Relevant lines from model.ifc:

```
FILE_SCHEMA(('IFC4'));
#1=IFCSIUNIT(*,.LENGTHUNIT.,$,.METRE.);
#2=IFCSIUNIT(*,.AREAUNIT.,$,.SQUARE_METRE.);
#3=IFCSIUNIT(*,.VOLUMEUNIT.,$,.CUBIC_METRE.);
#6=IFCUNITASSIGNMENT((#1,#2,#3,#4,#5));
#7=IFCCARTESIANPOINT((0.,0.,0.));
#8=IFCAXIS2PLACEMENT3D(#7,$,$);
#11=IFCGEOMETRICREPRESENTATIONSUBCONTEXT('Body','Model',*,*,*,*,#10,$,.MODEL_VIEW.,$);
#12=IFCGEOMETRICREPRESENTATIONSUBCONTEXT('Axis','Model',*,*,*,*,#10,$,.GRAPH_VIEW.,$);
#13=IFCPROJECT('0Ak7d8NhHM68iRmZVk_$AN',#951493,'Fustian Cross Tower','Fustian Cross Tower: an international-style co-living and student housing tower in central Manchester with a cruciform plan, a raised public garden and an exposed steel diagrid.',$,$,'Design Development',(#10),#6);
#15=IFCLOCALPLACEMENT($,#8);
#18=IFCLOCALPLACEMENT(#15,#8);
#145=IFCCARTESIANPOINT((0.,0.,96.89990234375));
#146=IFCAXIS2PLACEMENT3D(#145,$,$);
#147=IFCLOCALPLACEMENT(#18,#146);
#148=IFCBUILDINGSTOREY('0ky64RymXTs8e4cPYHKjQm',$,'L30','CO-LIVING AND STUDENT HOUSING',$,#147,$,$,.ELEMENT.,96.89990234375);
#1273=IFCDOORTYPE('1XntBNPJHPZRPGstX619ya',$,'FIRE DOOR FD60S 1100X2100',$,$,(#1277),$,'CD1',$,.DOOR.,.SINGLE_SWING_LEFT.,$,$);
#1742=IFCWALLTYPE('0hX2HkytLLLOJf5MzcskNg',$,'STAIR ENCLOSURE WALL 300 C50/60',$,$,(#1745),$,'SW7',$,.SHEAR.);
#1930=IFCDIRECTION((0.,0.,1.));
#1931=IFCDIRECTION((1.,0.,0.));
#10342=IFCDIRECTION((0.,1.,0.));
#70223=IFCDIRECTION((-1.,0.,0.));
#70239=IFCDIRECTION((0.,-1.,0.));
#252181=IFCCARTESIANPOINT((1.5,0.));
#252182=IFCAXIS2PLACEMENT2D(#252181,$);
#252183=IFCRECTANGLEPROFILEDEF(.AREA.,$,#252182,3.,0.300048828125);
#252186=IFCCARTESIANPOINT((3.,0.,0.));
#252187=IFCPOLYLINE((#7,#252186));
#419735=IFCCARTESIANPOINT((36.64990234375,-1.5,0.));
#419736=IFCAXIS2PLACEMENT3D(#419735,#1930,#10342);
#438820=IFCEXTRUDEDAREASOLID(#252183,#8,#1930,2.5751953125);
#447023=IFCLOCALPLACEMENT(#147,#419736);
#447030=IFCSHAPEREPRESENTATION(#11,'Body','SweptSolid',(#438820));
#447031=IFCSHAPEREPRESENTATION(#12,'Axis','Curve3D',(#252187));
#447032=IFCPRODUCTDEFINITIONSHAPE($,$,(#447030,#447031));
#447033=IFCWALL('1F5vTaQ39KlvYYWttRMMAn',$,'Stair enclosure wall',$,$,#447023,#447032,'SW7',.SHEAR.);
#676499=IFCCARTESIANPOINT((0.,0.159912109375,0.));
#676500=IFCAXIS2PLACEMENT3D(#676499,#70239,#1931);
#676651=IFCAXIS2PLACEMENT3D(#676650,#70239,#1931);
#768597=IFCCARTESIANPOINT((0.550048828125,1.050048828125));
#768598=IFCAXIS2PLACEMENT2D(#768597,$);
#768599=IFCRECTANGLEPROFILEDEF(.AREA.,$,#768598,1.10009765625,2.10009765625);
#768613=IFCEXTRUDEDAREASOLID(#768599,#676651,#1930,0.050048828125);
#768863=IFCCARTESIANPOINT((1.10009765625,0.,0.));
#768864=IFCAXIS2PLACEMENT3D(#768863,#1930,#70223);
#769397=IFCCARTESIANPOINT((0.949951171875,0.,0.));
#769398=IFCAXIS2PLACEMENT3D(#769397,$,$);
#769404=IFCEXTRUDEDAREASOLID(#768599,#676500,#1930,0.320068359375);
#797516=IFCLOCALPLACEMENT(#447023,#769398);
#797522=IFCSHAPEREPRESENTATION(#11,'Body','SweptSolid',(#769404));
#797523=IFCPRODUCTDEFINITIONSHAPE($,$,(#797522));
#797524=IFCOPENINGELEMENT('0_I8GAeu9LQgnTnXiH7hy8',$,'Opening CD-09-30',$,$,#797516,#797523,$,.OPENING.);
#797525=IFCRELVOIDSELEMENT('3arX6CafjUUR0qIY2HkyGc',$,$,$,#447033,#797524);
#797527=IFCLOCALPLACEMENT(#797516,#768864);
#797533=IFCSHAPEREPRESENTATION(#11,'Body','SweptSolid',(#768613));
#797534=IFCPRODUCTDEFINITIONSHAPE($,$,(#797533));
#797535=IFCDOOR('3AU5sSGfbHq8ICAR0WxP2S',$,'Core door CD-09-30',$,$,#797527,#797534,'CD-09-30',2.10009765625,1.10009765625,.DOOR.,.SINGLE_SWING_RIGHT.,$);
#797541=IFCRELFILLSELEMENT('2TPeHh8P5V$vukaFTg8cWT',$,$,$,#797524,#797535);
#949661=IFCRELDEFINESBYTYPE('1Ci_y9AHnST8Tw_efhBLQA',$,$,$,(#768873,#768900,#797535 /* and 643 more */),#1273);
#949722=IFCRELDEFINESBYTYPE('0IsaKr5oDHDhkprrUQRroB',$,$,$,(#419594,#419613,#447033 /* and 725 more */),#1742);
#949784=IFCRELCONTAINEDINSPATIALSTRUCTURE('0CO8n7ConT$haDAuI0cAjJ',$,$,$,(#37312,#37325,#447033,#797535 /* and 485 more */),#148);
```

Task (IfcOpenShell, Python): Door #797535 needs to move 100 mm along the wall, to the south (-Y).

```python
import ifcopenshell
import ifcopenshell.api.geometry
import ifcopenshell.util.placement
import ifcopenshell.util.unit

model = ifcopenshell.open("model.ifc")
unit_scale = ifcopenshell.util.unit.calculate_unit_scale(model)

door = model.by_guid("3AU5sSGfbHq8ICAR0WxP2S")
opening = door.FillsVoids[0].RelatingOpeningElement
wall = opening.VoidsElements[0].RelatingBuildingElement

wall_matrix = ifcopenshell.util.placement.get_local_placement(wall.ObjectPlacement)
shift = wall_matrix[:3, 0] * -0.1 / unit_scale
before = ifcopenshell.util.placement.get_local_placement(door.ObjectPlacement)[:3, 3].copy()

# The door is placed relative to its opening, so it follows when the opening moves.
matrix = ifcopenshell.util.placement.get_local_placement(opening.ObjectPlacement)
matrix[:3, 3] += shift
ifcopenshell.api.geometry.edit_object_placement(
    model, product=opening, matrix=matrix, is_si=False, should_transform_children=True
)

after = ifcopenshell.util.placement.get_local_placement(door.ObjectPlacement)[:3, 3]
print("door moved by", (after - before).round(3) + 0.0)

model.write("model-out.ifc")
```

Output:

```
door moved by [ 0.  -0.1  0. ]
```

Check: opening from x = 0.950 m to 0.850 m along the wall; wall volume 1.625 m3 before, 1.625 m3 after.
